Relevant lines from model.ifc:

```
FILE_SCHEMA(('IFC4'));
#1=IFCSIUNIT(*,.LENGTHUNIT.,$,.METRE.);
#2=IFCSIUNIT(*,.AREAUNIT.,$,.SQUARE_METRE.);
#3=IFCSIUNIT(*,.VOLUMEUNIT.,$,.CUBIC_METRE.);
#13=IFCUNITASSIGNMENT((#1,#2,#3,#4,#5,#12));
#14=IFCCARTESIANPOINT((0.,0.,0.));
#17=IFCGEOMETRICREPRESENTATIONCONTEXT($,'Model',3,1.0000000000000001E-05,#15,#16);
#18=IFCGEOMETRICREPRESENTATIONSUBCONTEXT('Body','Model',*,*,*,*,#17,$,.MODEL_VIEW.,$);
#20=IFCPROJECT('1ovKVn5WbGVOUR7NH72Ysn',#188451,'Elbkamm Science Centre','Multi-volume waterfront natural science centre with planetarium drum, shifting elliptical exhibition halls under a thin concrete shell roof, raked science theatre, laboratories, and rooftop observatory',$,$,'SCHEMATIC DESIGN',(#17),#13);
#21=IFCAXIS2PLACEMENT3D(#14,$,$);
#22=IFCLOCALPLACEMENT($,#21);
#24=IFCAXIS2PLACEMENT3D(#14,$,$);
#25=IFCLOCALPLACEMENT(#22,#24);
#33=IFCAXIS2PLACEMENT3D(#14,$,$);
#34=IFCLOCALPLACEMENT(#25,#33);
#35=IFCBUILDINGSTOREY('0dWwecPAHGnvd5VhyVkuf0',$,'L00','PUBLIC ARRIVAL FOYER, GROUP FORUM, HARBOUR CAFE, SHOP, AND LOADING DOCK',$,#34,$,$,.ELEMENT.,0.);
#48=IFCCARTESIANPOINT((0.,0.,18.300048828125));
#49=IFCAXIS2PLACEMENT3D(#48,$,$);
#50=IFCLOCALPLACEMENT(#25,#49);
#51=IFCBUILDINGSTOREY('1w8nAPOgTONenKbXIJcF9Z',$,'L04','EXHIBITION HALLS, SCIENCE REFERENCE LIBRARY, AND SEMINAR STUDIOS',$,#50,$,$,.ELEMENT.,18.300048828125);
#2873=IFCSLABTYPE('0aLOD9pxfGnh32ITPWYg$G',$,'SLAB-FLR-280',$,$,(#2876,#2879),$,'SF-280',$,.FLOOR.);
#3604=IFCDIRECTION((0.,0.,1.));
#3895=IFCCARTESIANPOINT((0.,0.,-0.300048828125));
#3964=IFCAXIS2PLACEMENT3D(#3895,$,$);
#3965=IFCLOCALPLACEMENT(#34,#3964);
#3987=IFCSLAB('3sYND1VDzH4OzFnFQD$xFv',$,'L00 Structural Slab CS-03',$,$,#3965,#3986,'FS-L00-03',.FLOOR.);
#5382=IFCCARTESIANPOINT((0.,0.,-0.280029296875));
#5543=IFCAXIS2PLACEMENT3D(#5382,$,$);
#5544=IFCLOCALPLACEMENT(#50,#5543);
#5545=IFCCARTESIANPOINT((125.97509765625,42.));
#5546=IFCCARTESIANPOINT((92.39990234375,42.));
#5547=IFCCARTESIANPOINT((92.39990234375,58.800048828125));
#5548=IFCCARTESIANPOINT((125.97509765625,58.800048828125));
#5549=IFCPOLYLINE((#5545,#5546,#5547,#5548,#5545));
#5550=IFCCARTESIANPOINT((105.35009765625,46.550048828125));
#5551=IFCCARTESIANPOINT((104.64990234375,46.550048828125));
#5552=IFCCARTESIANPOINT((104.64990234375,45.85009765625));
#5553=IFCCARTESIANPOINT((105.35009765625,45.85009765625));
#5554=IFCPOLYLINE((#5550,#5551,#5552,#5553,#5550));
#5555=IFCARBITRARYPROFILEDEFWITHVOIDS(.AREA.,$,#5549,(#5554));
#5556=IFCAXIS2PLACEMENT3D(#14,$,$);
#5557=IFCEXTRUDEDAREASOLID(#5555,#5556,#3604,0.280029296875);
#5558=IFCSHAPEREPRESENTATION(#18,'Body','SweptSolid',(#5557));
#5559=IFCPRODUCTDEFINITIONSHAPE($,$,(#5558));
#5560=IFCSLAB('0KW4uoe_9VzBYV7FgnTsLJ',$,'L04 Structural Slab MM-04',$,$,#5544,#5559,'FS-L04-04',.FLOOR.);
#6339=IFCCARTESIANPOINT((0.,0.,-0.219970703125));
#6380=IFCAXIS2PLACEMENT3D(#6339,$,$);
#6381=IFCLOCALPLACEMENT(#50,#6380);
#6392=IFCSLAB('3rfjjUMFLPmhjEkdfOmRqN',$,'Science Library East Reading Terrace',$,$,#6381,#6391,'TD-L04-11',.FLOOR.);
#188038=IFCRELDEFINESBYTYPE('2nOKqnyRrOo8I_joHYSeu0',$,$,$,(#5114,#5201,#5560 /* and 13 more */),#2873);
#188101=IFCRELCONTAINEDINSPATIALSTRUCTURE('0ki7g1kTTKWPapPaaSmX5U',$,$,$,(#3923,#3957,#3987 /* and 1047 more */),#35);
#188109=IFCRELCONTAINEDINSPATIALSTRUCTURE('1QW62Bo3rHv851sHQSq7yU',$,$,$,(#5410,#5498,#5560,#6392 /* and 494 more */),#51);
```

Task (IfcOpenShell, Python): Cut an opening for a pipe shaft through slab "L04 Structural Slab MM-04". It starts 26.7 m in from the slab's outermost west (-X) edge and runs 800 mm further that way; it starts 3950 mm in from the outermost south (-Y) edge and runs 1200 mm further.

```python
import numpy as np
import ifcopenshell
import ifcopenshell.api.feature
import ifcopenshell.api.geometry
import ifcopenshell.api.root
import ifcopenshell.geom
import ifcopenshell.util.placement
import ifcopenshell.util.representation
import ifcopenshell.util.shape
import ifcopenshell.util.unit

model = ifcopenshell.open("model.ifc")
unit_scale = ifcopenshell.util.unit.calculate_unit_scale(model)
settings = ifcopenshell.geom.settings()


def volume(element):
    """Net volume in cubic metres, openings subtracted."""
    shape = ifcopenshell.geom.create_shape(settings, element)
    return ifcopenshell.util.shape.get_volume(shape.geometry)


slab = model.by_id(5560)
before = volume(slab)

# Extent in the slab's own axes, in metres. The edges named are its -X and -Y sides.
slab_shape = ifcopenshell.geom.create_shape(settings, slab)
vertices = ifcopenshell.util.shape.get_vertices(slab_shape.geometry)
x_min, y_min, bottom = vertices.min(axis=0)
top = vertices[:, 2].max()

opening = ifcopenshell.api.root.create_entity(model, ifc_class="IfcOpeningElement", name="Pipe shaft opening", predefined_type="OPENING")
context = ifcopenshell.util.representation.get_context(model, "Model", "Body", "MODEL_VIEW")
width, depth = 0.8, 1.2
outline = [(0.0, 0.0), (width, 0.0), (width, depth), (0.0, depth), (0.0, 0.0)]
# Overshoot both faces by 50 mm so the cut is clean.
shape = ifcopenshell.api.geometry.add_slab_representation(
    model, context=context, depth=top - bottom + 0.1, polyline=outline
)
ifcopenshell.api.geometry.assign_representation(model, product=opening, representation=shape)

matrix = ifcopenshell.util.placement.get_local_placement(slab.ObjectPlacement)
matrix[:, 3] = matrix @ np.append(np.array([x_min + 26.7, y_min + 3.95, bottom - 0.05]) / unit_scale, 1.0)
ifcopenshell.api.geometry.edit_object_placement(model, product=opening, matrix=matrix, is_si=False)
ifcopenshell.api.feature.add_feature(model, feature=opening, element=slab)

after = volume(slab)

print(f"slab volume {before:.3f} -> {after:.3f} m3")

model.write("model-out.ifc")
```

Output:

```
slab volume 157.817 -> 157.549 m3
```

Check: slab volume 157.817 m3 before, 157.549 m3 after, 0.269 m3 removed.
